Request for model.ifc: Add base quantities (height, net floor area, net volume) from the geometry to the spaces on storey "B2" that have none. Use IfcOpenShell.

First a look at what the model holds.

```python
import ifcopenshell
import ifcopenshell.util.element
import ifcopenshell.util.unit

model = ifcopenshell.open("model.ifc")
print(model.schema)
for unit_type in ("LENGTHUNIT", "AREAUNIT", "VOLUMEUNIT"):
    print(unit_type, ifcopenshell.util.unit.calculate_unit_scale(model, unit_type))
storey = next(s for s in model.by_type("IfcBuildingStorey") if s.Name == "B2")
spaces = [e for e in ifcopenshell.util.element.get_decomposition(storey) if e.is_a("IfcSpace")]
for e in sorted(spaces, key=lambda e: e.id()):
    print(e.id(), e.is_a(), e.Name, list(ifcopenshell.util.element.get_psets(e, qtos_only=True)), sep=" | ")
```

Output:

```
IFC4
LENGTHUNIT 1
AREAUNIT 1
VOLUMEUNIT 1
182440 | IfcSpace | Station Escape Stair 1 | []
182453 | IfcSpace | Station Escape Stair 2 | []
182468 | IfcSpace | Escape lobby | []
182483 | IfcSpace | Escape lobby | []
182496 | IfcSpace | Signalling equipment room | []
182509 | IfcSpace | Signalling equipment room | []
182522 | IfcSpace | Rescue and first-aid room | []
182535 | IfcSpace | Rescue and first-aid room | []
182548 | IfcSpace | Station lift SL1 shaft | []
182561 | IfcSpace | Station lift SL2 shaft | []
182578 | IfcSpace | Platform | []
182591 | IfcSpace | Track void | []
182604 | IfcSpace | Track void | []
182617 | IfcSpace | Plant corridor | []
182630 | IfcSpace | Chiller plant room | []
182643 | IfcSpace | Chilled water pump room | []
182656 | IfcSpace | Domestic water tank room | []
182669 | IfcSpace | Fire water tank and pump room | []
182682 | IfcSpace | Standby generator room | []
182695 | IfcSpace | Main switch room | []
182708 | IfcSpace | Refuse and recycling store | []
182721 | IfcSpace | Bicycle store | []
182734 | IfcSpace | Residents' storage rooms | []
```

```python
import ifcopenshell
import ifcopenshell.api.pset
import ifcopenshell.geom
import ifcopenshell.util.element
import ifcopenshell.util.shape
import ifcopenshell.util.unit

model = ifcopenshell.open("model.ifc")
unit_scale = ifcopenshell.util.unit.calculate_unit_scale(model)
area_scale = ifcopenshell.util.unit.calculate_unit_scale(model, "AREAUNIT")
volume_scale = ifcopenshell.util.unit.calculate_unit_scale(model, "VOLUMEUNIT")
settings = ifcopenshell.geom.settings()

storey = next(s for s in model.by_type("IfcBuildingStorey") if s.Name == "B2")
spaces = [e for e in ifcopenshell.util.element.get_decomposition(storey) if e.is_a("IfcSpace")]

for e in sorted(spaces, key=lambda e: e.id()):
    if ifcopenshell.util.element.get_psets(e, qtos_only=True, should_inherit=False):
        continue
    # Geometry comes back in metres, in the element's own axes.
    shape = ifcopenshell.geom.create_shape(settings, e)
    values = {
        "Height": ifcopenshell.util.shape.get_z(shape.geometry) / unit_scale,
        "NetFloorArea": ifcopenshell.util.shape.get_footprint_area(shape.geometry) / area_scale,
        "NetVolume": ifcopenshell.util.shape.get_volume(shape.geometry) / volume_scale,
    }
    qto = ifcopenshell.api.pset.add_qto(model, product=e, name="Qto_SpaceBaseQuantities")
    ifcopenshell.api.pset.edit_qto(model, qto=qto, properties=values)
    print(e.id(), {k: round(v, 3) for k, v in values.items()})

model.write("model_rev.ifc")
```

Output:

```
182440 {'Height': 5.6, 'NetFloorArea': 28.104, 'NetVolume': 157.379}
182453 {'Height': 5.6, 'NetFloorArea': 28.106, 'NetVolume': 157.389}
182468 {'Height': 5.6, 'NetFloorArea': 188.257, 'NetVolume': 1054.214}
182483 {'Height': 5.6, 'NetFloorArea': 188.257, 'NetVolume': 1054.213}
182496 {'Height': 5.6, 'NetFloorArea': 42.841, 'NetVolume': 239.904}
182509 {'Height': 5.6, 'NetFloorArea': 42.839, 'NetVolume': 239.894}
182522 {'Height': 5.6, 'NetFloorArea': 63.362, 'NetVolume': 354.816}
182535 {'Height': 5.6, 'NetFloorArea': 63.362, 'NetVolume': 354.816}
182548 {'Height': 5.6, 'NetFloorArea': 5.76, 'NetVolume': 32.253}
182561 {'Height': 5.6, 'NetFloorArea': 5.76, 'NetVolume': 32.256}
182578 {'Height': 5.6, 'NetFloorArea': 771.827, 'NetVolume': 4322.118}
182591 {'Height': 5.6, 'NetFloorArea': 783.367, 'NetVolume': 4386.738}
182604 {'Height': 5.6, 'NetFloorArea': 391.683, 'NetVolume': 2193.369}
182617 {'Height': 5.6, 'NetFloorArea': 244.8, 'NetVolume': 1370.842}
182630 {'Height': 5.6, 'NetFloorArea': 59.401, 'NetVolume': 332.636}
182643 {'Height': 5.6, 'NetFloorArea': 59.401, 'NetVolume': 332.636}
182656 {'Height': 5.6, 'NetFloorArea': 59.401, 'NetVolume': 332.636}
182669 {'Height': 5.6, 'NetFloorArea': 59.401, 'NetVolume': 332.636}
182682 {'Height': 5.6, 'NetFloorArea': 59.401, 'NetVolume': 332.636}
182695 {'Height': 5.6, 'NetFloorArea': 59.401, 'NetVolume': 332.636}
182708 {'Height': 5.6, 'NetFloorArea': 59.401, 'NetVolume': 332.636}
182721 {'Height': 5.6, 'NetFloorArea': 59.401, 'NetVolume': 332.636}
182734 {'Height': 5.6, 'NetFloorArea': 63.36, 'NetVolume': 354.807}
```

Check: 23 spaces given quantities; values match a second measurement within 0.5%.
